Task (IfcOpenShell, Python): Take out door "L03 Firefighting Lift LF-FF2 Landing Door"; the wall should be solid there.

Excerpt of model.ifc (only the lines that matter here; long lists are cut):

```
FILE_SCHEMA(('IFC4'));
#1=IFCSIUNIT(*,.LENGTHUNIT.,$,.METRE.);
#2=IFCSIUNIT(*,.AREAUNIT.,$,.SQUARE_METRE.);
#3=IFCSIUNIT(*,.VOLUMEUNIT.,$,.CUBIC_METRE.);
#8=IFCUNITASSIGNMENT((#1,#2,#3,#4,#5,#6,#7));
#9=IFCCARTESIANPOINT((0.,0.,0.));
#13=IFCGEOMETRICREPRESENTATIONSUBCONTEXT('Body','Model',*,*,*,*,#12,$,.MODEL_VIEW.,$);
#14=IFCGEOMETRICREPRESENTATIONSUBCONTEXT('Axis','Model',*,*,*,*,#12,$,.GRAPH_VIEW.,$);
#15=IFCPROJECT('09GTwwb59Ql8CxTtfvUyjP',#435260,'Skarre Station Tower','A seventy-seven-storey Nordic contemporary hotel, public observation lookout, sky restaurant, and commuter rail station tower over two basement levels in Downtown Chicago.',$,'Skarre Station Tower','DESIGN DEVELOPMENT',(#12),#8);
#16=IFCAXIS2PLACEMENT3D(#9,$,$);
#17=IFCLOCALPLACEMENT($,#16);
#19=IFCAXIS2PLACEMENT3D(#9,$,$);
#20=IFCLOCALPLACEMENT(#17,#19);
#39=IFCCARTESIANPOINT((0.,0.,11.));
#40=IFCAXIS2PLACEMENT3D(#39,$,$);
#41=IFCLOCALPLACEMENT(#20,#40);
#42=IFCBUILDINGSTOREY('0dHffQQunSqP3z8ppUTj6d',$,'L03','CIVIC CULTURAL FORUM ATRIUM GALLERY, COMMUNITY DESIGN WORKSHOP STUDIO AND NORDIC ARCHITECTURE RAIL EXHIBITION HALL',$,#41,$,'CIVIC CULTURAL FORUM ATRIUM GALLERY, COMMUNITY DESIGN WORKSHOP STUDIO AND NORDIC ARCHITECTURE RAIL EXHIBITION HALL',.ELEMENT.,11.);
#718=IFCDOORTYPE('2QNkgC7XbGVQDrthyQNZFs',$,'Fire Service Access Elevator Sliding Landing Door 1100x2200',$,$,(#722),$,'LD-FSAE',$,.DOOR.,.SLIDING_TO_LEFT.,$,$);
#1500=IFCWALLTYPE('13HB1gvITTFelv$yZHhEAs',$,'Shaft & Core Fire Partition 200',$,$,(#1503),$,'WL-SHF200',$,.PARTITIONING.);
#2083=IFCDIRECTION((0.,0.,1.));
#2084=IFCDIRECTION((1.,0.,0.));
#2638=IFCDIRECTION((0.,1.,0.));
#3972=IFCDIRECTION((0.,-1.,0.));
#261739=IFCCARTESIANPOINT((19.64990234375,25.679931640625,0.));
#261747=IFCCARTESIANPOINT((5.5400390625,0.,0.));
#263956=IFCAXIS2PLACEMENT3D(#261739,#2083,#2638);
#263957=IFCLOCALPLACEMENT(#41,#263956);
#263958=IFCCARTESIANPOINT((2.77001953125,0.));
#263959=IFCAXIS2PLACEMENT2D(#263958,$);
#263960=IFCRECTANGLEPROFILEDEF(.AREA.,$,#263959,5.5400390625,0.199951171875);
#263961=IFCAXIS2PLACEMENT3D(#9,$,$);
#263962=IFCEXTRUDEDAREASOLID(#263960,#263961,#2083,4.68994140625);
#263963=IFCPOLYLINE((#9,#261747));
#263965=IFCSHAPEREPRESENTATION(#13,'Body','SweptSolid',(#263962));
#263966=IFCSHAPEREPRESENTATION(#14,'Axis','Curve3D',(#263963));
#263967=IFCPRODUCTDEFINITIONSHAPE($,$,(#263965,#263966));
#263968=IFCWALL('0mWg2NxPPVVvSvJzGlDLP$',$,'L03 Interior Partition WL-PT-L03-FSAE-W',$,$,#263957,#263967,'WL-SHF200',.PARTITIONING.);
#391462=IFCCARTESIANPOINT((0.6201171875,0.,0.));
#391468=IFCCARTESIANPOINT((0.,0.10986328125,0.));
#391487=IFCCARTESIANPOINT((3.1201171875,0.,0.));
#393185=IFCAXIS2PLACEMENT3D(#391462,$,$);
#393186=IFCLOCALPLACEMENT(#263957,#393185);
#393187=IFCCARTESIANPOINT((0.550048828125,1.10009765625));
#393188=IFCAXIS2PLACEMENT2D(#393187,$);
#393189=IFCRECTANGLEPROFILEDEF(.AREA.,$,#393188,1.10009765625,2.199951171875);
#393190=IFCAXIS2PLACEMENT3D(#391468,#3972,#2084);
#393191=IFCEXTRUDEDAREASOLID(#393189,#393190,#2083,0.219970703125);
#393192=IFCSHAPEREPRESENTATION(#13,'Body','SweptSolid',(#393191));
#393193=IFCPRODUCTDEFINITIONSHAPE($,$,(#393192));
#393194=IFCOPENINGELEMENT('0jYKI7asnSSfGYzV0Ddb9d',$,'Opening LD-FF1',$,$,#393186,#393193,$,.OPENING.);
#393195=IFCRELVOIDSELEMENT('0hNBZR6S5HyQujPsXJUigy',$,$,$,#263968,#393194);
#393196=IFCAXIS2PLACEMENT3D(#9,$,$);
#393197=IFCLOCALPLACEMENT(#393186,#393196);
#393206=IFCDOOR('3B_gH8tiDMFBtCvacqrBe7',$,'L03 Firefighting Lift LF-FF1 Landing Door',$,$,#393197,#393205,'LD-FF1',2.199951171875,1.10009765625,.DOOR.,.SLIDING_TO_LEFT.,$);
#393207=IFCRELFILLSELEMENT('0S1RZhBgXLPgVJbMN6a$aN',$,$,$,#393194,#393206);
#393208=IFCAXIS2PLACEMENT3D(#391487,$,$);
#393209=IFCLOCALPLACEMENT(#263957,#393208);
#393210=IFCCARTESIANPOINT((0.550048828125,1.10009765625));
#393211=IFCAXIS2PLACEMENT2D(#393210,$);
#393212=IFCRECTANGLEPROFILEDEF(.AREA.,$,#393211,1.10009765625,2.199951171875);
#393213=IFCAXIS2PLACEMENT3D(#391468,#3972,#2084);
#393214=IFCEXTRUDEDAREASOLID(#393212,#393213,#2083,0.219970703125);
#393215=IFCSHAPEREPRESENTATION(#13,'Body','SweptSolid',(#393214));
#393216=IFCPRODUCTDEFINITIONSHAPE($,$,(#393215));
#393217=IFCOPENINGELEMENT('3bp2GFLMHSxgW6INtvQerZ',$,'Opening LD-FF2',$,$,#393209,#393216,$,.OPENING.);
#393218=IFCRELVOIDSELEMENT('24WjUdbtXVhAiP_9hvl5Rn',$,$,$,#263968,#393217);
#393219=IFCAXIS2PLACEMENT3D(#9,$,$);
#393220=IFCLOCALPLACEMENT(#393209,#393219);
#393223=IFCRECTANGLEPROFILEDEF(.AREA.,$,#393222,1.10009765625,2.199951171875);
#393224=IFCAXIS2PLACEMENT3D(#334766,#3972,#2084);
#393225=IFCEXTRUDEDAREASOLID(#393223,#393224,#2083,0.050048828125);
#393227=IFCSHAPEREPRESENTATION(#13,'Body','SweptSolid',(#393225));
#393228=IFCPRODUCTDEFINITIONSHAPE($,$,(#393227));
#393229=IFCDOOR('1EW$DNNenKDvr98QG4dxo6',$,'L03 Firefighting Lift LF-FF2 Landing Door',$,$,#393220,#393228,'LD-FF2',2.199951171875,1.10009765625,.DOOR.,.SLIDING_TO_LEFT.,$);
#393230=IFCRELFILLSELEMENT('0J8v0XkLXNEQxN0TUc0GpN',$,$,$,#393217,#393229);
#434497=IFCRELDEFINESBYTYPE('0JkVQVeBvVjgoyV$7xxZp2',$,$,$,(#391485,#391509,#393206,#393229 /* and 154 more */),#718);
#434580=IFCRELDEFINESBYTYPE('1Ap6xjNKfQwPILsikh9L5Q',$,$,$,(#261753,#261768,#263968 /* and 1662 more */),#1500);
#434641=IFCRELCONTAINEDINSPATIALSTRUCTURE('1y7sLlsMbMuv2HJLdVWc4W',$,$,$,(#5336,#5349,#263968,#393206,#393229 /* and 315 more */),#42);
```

```python
import ifcopenshell
import ifcopenshell.api.feature
import ifcopenshell.api.root
import ifcopenshell.geom
import ifcopenshell.util.shape

model = ifcopenshell.open("model.ifc")
settings = ifcopenshell.geom.settings()


def volume(element):
    """Net volume in cubic metres, openings subtracted."""
    shape = ifcopenshell.geom.create_shape(settings, element)
    return ifcopenshell.util.shape.get_volume(shape.geometry)


door = model.by_id(393229)
opening = door.FillsVoids[0].RelatingOpeningElement
wall = opening.VoidsElements[0].RelatingBuildingElement
before = volume(wall)

ifcopenshell.api.root.remove_product(model, product=door)
ifcopenshell.api.feature.remove_feature(model, feature=opening)

after = volume(wall)

print(f"wall volume {before:.3f} -> {after:.3f} m3")

model.write("model_rev.ifc")
```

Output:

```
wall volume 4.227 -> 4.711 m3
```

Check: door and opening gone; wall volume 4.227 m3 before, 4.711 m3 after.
